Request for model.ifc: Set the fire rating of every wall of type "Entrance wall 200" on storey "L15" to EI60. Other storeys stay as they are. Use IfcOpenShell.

First a look at what the model holds.

```python
import ifcopenshell
import ifcopenshell.util.element

model = ifcopenshell.open("model.ifc")
print(model.schema)
storey = next(s for s in model.by_type("IfcBuildingStorey") if s.Name == "L15")
walls = [e for e in ifcopenshell.util.element.get_decomposition(storey) if e.is_a("IfcWall")]
seen = {}
for e in walls:
    element_type = ifcopenshell.util.element.get_type(e)
    key = (element_type.Name if element_type != e and element_type else None, ifcopenshell.util.element.get_pset(e, "Pset_WallCommon", "FireRating"))
    seen[key] = seen.get(key, 0) + 1
for (name, value), count in sorted(seen.items(), key=str):
    print(count, "x", name, "|", value)
```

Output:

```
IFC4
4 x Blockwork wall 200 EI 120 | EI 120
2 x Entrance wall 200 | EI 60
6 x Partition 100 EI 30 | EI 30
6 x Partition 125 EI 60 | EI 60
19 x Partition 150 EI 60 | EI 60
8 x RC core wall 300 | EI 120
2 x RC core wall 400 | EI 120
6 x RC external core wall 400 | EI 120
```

```python
import ifcopenshell
import ifcopenshell.api.pset
import ifcopenshell.util.element

model = ifcopenshell.open("model.ifc")

storey = next(s for s in model.by_type("IfcBuildingStorey") if s.Name == "L15")
walls = [e for e in ifcopenshell.util.element.get_decomposition(storey) if e.is_a("IfcWall")]

count = 0
for e in walls:
    element_type = ifcopenshell.util.element.get_type(e)
    if element_type in (None, e) or element_type.Name != "Entrance wall 200":
        continue
    # add_pset returns the element's existing set when there is one.
    pset = ifcopenshell.api.pset.add_pset(model, product=e, name="Pset_WallCommon")
    ifcopenshell.api.pset.edit_pset(model, pset=pset, properties={"FireRating": "EI60"})
    count += 1

print(count, "walls updated")

model.write("model_edited.ifc")
```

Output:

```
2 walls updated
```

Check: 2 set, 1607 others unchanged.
